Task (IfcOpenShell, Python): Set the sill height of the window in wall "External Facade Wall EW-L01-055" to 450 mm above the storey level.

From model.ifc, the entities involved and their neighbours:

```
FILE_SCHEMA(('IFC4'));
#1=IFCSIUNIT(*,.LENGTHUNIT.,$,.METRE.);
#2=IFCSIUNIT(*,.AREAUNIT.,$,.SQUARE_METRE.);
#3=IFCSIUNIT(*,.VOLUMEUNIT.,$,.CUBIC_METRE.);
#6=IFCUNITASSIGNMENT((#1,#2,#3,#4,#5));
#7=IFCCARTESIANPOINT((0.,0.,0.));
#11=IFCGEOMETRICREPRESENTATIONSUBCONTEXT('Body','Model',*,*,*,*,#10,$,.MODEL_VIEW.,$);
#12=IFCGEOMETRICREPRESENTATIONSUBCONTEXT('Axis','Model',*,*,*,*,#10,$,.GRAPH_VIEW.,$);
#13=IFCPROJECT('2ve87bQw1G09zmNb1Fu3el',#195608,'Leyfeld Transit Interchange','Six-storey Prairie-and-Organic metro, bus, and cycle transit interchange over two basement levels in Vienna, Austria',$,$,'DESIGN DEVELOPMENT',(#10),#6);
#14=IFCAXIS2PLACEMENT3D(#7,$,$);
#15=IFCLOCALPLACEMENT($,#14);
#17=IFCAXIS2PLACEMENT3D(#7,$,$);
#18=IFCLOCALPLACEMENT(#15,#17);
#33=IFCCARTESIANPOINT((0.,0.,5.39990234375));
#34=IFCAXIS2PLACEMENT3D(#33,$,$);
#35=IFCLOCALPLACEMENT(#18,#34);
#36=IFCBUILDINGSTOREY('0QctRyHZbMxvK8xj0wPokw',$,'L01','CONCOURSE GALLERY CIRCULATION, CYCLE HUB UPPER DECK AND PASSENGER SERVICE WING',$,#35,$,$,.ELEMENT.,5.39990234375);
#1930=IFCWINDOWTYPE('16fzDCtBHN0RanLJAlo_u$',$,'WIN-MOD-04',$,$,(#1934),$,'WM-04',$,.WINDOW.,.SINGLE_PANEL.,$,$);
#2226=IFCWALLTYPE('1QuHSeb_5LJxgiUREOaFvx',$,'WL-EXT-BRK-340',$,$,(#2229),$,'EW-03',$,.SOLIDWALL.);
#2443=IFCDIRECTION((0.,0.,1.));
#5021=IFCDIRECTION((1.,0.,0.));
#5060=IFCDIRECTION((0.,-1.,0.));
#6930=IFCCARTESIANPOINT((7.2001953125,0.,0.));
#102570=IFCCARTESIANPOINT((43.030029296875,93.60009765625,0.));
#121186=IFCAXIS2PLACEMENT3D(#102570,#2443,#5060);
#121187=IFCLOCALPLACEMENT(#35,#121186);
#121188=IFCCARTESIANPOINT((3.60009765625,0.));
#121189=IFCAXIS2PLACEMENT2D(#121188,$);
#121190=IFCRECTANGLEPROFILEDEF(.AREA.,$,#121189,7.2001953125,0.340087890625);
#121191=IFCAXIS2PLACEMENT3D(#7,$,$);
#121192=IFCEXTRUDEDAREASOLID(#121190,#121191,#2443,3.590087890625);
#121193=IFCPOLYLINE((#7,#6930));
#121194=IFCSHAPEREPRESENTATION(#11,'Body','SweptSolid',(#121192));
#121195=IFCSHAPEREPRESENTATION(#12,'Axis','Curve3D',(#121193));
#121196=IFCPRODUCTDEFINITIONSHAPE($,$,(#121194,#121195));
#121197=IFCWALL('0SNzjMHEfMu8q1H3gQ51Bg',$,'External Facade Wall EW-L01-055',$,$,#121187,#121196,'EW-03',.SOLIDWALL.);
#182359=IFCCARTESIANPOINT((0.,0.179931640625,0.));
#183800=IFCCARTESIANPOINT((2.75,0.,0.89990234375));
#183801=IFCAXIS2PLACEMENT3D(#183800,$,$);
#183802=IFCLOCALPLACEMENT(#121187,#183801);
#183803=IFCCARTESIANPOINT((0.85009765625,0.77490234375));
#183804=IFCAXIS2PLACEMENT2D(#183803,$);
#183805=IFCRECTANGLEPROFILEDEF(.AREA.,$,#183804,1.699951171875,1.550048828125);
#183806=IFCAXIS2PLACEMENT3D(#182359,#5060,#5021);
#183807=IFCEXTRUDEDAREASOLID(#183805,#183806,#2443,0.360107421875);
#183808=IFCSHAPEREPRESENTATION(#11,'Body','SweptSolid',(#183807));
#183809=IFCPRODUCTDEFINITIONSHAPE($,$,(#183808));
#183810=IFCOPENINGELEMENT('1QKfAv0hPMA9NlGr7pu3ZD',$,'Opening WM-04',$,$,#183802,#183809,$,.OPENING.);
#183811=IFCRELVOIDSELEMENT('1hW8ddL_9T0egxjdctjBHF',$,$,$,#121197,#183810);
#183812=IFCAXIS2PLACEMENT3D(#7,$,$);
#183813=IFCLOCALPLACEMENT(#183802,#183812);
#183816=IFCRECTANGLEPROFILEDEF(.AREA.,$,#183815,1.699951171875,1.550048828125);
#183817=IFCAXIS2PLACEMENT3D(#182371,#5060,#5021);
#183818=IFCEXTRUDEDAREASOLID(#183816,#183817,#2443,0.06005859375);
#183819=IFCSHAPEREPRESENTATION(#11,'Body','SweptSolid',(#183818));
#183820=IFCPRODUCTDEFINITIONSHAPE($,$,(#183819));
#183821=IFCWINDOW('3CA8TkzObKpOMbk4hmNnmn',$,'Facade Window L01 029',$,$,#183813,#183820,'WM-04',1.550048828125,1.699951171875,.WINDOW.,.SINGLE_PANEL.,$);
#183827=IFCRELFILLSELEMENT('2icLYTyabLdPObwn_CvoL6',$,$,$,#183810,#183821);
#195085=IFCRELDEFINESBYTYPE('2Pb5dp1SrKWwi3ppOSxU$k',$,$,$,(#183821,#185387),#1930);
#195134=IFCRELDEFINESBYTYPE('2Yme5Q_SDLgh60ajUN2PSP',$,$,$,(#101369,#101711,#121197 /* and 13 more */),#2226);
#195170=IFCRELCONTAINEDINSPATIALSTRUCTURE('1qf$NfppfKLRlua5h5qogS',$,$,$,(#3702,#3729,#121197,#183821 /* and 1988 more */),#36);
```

```python
import numpy as np
import ifcopenshell
import ifcopenshell.api.geometry
import ifcopenshell.geom
import ifcopenshell.util.element
import ifcopenshell.util.placement
import ifcopenshell.util.shape
import ifcopenshell.util.unit

model = ifcopenshell.open("model.ifc")
unit_scale = ifcopenshell.util.unit.calculate_unit_scale(model)

window = model.by_id(183821)
opening = window.FillsVoids[0].RelatingOpeningElement
storey = ifcopenshell.util.element.get_container(window, ifc_class="IfcBuildingStorey")
level = ifcopenshell.util.placement.get_local_placement(storey.ObjectPlacement)[2, 3]

# The opening's origin need not be at the sill, so measure its lowest point.
shape = ifcopenshell.geom.create_shape(ifcopenshell.geom.settings(), opening)
bottom = ifcopenshell.util.shape.get_shape_bottom_elevation(shape, shape.geometry) / unit_scale
dz = level + 0.45 / unit_scale - bottom

shift = np.array([0.0, 0.0, dz])
# The window is placed relative to its opening, so it follows when the opening moves.
matrix = ifcopenshell.util.placement.get_local_placement(opening.ObjectPlacement)
matrix[:3, 3] += shift
ifcopenshell.api.geometry.edit_object_placement(
    model, product=opening, matrix=matrix, is_si=False, should_transform_children=True
)

print(f"moved by {dz * unit_scale:+.3f} m")

model.write("model_updated.ifc")
```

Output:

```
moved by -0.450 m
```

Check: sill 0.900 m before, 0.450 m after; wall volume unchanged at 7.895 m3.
